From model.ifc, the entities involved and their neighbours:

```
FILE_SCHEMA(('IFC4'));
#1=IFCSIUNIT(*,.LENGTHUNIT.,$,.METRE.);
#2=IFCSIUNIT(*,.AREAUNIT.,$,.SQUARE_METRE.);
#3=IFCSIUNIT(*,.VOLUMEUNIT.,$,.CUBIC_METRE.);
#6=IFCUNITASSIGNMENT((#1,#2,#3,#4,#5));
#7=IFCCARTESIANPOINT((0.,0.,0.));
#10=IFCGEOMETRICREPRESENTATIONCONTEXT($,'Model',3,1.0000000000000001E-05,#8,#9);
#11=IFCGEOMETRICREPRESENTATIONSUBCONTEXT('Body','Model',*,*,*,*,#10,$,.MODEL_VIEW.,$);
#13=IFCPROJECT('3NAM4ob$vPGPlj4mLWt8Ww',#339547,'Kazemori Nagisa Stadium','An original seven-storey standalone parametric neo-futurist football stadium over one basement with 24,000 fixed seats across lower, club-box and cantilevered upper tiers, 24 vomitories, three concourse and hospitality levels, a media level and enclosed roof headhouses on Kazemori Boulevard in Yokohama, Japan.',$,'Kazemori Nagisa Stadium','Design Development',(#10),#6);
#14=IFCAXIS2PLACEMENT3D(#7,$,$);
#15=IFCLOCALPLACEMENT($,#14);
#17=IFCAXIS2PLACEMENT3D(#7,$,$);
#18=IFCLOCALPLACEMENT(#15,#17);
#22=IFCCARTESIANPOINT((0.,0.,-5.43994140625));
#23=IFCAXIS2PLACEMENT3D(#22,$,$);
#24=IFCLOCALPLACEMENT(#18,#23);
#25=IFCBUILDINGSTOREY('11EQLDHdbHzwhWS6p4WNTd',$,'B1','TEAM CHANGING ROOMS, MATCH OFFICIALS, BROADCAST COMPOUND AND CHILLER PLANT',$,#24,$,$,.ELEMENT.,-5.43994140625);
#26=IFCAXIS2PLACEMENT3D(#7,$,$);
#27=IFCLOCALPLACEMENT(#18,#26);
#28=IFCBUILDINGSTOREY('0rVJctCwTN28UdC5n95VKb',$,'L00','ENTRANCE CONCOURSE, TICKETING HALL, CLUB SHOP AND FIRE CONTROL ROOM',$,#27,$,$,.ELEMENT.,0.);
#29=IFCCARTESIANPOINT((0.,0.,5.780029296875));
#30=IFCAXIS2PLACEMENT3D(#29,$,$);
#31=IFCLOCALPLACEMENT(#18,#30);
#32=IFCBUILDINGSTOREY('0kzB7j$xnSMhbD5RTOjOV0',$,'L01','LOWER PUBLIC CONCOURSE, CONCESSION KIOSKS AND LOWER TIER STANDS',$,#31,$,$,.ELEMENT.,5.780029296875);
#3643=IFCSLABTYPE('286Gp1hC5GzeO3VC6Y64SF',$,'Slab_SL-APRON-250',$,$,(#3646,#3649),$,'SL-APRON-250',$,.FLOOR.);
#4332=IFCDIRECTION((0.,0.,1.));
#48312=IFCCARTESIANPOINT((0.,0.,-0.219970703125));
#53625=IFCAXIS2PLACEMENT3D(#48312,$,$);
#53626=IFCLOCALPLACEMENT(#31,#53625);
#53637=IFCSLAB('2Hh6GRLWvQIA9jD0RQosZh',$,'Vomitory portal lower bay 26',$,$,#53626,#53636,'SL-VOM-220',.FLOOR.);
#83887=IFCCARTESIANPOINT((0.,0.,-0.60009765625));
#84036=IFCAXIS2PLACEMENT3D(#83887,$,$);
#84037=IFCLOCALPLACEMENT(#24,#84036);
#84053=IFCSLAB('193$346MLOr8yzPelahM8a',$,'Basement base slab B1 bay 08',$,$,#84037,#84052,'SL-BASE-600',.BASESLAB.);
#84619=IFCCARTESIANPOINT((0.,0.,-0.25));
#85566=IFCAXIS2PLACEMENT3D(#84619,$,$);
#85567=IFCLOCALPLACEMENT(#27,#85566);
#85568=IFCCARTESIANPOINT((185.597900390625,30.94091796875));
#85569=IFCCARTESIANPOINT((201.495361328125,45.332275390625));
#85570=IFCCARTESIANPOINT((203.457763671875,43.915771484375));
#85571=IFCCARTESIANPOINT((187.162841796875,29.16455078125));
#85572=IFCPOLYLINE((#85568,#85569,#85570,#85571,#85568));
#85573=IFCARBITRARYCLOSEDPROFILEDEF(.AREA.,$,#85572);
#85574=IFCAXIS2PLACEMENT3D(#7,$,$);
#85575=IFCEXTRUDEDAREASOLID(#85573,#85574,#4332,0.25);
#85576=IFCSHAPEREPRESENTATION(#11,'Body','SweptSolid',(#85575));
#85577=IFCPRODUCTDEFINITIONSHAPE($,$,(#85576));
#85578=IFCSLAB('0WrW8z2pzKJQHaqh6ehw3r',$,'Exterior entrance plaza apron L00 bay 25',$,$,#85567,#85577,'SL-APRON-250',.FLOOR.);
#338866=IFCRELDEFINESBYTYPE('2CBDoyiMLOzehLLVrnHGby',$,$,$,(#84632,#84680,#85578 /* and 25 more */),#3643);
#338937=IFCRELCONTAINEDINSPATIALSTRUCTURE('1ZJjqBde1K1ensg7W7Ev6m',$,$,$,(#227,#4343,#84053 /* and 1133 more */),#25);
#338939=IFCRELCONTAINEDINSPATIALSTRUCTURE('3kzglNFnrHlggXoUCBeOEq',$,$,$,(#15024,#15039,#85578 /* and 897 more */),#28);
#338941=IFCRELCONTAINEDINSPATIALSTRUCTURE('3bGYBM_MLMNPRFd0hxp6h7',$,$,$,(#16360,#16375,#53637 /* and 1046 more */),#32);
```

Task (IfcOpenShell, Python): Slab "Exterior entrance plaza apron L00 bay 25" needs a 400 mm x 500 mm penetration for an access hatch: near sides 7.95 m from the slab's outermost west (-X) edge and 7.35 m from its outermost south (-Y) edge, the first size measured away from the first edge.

```python
import numpy as np
import ifcopenshell
import ifcopenshell.api.feature
import ifcopenshell.api.geometry
import ifcopenshell.api.root
import ifcopenshell.geom
import ifcopenshell.util.placement
import ifcopenshell.util.representation
import ifcopenshell.util.shape
import ifcopenshell.util.unit

model = ifcopenshell.open("model.ifc")
unit_scale = ifcopenshell.util.unit.calculate_unit_scale(model)
settings = ifcopenshell.geom.settings()


def volume(element):
    """Net volume in cubic metres, openings subtracted."""
    shape = ifcopenshell.geom.create_shape(settings, element)
    return ifcopenshell.util.shape.get_volume(shape.geometry)


slab = model.by_guid("0WrW8z2pzKJQHaqh6ehw3r")
before = volume(slab)

# Extent in the slab's own axes, in metres. The edges named are its -X and -Y sides.
slab_shape = ifcopenshell.geom.create_shape(settings, slab)
vertices = ifcopenshell.util.shape.get_vertices(slab_shape.geometry)
x_min, y_min, bottom = vertices.min(axis=0)
top = vertices[:, 2].max()

opening = ifcopenshell.api.root.create_entity(model, ifc_class="IfcOpeningElement", name="Access hatch opening", predefined_type="OPENING")
context = ifcopenshell.util.representation.get_context(model, "Model", "Body", "MODEL_VIEW")
width, depth = 0.4, 0.5
outline = [(0.0, 0.0), (width, 0.0), (width, depth), (0.0, depth), (0.0, 0.0)]
# Overshoot both faces by 50 mm so the cut is clean.
shape = ifcopenshell.api.geometry.add_slab_representation(
    model, context=context, depth=top - bottom + 0.1, polyline=outline
)
ifcopenshell.api.geometry.assign_representation(model, product=opening, representation=shape)

matrix = ifcopenshell.util.placement.get_local_placement(slab.ObjectPlacement)
matrix[:, 3] = matrix @ np.append(np.array([x_min + 7.95, y_min + 7.35, bottom - 0.05]) / unit_scale, 1.0)
ifcopenshell.api.geometry.edit_object_placement(model, product=opening, matrix=matrix, is_si=False)
ifcopenshell.api.feature.add_feature(model, feature=opening, element=slab)

after = volume(slab)

print(f"slab volume {before:.3f} -> {after:.3f} m3")

model.write("model-out.ifc")
```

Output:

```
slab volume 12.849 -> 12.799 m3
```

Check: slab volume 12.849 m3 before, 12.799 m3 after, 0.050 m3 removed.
